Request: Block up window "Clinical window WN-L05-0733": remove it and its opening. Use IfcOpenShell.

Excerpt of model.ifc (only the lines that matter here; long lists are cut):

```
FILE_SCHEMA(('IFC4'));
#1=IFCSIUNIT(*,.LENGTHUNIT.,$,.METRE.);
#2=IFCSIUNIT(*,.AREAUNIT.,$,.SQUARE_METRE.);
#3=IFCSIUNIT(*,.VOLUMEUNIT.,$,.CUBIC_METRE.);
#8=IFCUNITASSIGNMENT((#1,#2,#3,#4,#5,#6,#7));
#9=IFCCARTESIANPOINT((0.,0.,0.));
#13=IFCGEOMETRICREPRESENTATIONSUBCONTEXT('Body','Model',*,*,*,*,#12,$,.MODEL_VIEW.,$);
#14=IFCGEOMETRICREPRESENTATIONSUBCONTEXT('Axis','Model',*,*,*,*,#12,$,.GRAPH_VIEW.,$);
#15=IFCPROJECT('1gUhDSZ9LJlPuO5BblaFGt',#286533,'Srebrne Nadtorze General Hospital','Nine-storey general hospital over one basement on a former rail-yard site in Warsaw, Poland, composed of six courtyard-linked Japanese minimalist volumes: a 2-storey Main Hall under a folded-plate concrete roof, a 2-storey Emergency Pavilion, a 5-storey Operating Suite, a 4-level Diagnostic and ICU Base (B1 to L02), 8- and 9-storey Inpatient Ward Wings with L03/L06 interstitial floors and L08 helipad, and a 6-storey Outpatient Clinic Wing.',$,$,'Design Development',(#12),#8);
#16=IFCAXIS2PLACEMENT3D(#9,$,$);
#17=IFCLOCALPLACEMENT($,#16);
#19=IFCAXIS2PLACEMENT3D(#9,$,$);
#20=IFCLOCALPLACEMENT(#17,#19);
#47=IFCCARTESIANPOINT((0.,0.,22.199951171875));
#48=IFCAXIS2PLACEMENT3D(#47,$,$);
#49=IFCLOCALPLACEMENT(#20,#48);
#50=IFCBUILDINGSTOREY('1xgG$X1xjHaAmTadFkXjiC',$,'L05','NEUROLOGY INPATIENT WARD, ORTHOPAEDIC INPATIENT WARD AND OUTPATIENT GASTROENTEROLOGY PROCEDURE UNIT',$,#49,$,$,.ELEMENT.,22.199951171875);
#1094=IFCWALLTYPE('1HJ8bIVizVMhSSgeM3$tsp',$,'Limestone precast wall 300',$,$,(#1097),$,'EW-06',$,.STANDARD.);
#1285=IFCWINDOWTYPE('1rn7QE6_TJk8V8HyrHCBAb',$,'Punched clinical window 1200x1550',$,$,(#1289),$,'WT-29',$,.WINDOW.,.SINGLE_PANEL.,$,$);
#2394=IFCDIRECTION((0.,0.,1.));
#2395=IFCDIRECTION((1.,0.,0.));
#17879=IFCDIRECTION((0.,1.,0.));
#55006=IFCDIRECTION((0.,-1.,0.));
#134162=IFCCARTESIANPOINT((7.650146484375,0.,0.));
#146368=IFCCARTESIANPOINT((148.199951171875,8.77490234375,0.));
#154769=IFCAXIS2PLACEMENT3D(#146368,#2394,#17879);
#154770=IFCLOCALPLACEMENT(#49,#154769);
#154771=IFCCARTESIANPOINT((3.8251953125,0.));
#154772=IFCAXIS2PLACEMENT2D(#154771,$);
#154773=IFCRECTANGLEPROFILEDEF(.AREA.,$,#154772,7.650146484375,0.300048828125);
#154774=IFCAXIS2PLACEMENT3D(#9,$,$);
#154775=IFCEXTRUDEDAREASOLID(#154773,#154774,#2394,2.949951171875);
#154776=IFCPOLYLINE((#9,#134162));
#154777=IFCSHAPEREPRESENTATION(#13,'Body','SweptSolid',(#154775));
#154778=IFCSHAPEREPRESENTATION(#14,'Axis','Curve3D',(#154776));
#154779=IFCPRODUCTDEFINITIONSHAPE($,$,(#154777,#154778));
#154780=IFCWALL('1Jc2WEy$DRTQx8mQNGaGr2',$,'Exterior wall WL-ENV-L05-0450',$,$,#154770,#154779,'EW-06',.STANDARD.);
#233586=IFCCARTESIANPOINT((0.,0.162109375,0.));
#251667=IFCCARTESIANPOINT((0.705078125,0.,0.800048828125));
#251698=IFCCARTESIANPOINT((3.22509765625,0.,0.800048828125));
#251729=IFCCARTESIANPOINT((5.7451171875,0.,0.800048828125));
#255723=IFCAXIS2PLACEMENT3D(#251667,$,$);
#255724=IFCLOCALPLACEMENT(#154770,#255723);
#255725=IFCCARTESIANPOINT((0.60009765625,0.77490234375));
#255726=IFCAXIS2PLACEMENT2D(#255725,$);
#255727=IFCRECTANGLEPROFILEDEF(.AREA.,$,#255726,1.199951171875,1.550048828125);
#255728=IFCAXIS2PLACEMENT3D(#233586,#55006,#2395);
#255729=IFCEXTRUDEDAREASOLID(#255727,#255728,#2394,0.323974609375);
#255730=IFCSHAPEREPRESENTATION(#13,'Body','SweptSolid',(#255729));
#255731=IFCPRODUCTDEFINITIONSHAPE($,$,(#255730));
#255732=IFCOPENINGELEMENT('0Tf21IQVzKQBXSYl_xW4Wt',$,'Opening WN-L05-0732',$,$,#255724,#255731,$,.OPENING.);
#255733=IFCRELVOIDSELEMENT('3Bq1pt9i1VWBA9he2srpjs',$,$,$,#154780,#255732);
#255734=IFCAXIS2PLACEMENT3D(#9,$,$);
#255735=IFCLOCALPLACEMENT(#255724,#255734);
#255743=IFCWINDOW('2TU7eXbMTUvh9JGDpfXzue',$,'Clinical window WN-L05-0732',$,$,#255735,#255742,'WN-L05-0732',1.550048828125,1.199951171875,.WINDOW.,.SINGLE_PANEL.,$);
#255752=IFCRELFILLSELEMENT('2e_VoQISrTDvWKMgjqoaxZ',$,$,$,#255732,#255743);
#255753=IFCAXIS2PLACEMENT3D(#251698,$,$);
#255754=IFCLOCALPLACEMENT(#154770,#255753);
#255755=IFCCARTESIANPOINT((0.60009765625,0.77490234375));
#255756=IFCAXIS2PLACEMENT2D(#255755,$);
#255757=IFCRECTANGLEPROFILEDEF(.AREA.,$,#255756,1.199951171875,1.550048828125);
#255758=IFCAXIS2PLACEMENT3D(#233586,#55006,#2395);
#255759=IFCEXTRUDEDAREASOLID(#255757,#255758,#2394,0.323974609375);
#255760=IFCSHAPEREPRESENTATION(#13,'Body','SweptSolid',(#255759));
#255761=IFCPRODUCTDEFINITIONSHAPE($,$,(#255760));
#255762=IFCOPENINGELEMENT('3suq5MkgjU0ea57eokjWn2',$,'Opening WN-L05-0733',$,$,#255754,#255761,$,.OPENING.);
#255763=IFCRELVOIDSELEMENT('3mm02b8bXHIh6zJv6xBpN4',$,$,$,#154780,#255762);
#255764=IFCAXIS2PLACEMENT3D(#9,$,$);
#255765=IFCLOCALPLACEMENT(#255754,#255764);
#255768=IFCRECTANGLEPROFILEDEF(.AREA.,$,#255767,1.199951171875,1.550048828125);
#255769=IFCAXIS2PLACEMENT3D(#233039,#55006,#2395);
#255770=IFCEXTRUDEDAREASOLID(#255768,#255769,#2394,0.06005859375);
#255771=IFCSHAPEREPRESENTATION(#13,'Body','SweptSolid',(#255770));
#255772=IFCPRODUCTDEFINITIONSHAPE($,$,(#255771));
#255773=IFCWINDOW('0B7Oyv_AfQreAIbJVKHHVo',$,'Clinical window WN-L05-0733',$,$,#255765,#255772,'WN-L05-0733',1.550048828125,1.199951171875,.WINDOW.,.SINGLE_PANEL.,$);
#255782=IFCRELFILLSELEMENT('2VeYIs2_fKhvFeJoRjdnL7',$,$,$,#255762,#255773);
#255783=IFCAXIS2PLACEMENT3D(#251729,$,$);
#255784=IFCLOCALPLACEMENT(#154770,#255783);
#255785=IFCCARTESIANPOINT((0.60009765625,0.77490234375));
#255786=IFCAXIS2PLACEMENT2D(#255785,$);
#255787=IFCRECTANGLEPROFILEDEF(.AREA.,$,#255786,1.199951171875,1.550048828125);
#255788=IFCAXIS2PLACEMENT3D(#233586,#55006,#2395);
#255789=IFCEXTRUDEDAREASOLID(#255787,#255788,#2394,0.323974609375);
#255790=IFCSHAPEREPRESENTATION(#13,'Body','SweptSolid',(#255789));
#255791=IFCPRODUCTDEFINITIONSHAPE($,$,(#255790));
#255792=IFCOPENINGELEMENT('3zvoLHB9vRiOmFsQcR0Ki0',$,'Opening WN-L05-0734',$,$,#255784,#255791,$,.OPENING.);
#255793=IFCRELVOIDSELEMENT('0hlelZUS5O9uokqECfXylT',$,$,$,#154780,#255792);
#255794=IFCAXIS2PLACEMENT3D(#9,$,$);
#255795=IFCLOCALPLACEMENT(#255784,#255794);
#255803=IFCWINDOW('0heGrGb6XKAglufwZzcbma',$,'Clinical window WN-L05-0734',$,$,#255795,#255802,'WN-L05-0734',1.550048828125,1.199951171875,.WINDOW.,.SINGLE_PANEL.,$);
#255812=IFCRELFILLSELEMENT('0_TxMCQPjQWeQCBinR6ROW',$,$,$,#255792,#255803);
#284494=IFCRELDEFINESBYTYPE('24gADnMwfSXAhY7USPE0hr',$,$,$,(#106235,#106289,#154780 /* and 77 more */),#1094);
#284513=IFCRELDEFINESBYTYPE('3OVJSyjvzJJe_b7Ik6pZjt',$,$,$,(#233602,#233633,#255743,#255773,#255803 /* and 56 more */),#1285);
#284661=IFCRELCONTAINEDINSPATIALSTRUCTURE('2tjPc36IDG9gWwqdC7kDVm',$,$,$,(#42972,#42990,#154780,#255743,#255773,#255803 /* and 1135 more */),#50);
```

```python
import ifcopenshell
import ifcopenshell.api.feature
import ifcopenshell.api.root
import ifcopenshell.geom
import ifcopenshell.util.shape

model = ifcopenshell.open("model.ifc")
settings = ifcopenshell.geom.settings()


def volume(element):
    """Net volume in cubic metres, openings subtracted."""
    shape = ifcopenshell.geom.create_shape(settings, element)
    return ifcopenshell.util.shape.get_volume(shape.geometry)


window = model.by_guid("0B7Oyv_AfQreAIbJVKHHVo")
opening = window.FillsVoids[0].RelatingOpeningElement
wall = opening.VoidsElements[0].RelatingBuildingElement
before = volume(wall)

ifcopenshell.api.root.remove_product(model, product=window)
ifcopenshell.api.feature.remove_feature(model, feature=opening)

after = volume(wall)

print(f"wall volume {before:.3f} -> {after:.3f} m3")

model.write("model_edited.ifc")
```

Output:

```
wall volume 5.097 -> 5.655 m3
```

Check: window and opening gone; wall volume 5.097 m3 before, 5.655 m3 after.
